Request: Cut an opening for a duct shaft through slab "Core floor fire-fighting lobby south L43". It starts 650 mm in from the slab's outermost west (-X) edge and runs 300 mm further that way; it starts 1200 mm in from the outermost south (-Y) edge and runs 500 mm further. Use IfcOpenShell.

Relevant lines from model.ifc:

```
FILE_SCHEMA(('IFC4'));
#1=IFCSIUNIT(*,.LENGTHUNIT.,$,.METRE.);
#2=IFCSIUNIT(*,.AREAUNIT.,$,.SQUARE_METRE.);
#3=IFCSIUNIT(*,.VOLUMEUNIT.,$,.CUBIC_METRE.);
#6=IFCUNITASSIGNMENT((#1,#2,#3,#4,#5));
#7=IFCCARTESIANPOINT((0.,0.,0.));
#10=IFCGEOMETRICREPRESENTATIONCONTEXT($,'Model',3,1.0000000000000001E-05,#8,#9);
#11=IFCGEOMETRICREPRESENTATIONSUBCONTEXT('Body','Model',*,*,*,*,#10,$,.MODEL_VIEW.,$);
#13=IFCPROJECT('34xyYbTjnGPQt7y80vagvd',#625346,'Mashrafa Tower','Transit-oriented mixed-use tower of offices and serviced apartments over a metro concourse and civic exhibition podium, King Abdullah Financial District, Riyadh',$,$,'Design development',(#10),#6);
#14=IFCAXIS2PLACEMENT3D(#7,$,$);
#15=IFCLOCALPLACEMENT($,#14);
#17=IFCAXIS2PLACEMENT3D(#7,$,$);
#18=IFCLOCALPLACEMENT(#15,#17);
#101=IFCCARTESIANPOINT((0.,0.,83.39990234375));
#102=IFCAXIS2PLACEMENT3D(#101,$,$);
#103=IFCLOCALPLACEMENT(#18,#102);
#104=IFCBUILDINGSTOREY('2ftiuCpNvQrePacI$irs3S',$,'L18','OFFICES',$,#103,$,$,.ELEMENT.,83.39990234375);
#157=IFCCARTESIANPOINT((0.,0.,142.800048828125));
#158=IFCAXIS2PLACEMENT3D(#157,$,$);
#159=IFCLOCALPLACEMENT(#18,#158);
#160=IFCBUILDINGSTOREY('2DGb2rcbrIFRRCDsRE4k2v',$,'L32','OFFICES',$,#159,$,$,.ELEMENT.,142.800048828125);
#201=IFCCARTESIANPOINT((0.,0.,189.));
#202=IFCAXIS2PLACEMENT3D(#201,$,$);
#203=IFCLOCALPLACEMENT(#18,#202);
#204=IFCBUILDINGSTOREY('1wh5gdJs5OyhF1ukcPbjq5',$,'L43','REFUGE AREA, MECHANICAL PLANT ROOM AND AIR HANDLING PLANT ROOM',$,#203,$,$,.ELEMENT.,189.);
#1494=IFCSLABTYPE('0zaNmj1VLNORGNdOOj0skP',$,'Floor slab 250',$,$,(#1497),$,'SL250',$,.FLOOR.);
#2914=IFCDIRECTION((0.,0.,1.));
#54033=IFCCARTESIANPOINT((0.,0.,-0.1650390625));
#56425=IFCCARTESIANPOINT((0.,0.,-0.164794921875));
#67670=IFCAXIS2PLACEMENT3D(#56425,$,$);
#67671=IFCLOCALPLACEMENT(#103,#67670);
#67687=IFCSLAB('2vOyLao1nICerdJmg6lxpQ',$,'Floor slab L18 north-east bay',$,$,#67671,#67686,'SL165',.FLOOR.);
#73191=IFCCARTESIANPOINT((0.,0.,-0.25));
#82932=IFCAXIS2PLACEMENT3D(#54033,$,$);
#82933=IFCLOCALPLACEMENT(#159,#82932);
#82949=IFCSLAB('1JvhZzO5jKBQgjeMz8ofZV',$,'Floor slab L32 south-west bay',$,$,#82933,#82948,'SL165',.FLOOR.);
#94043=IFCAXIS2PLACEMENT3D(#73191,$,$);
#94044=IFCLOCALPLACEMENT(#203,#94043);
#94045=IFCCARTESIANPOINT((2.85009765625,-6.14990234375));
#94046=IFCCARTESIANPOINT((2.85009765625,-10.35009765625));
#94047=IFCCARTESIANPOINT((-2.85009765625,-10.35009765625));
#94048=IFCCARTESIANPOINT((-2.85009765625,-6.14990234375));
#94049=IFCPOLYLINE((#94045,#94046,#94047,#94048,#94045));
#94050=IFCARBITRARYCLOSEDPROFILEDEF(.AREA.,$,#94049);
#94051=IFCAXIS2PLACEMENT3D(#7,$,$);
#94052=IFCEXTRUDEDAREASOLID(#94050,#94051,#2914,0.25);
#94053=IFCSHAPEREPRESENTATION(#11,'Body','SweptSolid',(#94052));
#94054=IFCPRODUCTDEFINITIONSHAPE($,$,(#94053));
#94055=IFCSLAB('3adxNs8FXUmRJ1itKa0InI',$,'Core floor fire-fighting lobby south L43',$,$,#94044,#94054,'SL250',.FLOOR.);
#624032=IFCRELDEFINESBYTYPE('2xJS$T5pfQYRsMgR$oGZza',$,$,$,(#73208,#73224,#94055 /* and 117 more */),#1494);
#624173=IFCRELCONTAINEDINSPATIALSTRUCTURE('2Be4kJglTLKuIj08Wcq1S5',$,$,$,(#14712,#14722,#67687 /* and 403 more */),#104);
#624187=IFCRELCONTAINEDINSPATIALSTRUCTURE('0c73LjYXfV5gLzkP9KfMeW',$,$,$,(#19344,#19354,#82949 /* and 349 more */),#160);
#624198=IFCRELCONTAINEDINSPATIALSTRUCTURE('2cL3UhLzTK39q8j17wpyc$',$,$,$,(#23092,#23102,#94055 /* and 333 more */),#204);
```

```python
import numpy as np
import ifcopenshell
import ifcopenshell.api.feature
import ifcopenshell.api.geometry
import ifcopenshell.api.root
import ifcopenshell.geom
import ifcopenshell.util.placement
import ifcopenshell.util.representation
import ifcopenshell.util.shape
import ifcopenshell.util.unit

model = ifcopenshell.open("model.ifc")
unit_scale = ifcopenshell.util.unit.calculate_unit_scale(model)
settings = ifcopenshell.geom.settings()


def volume(element):
    """Net volume in cubic metres, openings subtracted."""
    shape = ifcopenshell.geom.create_shape(settings, element)
    return ifcopenshell.util.shape.get_volume(shape.geometry)


slab = model.by_guid("3adxNs8FXUmRJ1itKa0InI")
before = volume(slab)

# Extent in the slab's own axes, in metres. The edges named are its -X and -Y sides.
slab_shape = ifcopenshell.geom.create_shape(settings, slab)
vertices = ifcopenshell.util.shape.get_vertices(slab_shape.geometry)
x_min, y_min, bottom = vertices.min(axis=0)
top = vertices[:, 2].max()

opening = ifcopenshell.api.root.create_entity(model, ifc_class="IfcOpeningElement", name="Duct shaft opening", predefined_type="OPENING")
context = ifcopenshell.util.representation.get_context(model, "Model", "Body", "MODEL_VIEW")
width, depth = 0.3, 0.5
outline = [(0.0, 0.0), (width, 0.0), (width, depth), (0.0, depth), (0.0, 0.0)]
# Overshoot both faces by 50 mm so the cut is clean.
shape = ifcopenshell.api.geometry.add_slab_representation(
    model, context=context, depth=top - bottom + 0.1, polyline=outline
)
ifcopenshell.api.geometry.assign_representation(model, product=opening, representation=shape)

matrix = ifcopenshell.util.placement.get_local_placement(slab.ObjectPlacement)
matrix[:, 3] = matrix @ np.append(np.array([x_min + 0.65, y_min + 1.2, bottom - 0.05]) / unit_scale, 1.0)
ifcopenshell.api.geometry.edit_object_placement(model, product=opening, matrix=matrix, is_si=False)
ifcopenshell.api.feature.add_feature(model, feature=opening, element=slab)

after = volume(slab)

print(f"slab volume {before:.3f} -> {after:.3f} m3")

model.write("model_updated.ifc")
```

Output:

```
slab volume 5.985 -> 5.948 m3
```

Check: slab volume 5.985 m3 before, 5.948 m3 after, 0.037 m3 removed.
